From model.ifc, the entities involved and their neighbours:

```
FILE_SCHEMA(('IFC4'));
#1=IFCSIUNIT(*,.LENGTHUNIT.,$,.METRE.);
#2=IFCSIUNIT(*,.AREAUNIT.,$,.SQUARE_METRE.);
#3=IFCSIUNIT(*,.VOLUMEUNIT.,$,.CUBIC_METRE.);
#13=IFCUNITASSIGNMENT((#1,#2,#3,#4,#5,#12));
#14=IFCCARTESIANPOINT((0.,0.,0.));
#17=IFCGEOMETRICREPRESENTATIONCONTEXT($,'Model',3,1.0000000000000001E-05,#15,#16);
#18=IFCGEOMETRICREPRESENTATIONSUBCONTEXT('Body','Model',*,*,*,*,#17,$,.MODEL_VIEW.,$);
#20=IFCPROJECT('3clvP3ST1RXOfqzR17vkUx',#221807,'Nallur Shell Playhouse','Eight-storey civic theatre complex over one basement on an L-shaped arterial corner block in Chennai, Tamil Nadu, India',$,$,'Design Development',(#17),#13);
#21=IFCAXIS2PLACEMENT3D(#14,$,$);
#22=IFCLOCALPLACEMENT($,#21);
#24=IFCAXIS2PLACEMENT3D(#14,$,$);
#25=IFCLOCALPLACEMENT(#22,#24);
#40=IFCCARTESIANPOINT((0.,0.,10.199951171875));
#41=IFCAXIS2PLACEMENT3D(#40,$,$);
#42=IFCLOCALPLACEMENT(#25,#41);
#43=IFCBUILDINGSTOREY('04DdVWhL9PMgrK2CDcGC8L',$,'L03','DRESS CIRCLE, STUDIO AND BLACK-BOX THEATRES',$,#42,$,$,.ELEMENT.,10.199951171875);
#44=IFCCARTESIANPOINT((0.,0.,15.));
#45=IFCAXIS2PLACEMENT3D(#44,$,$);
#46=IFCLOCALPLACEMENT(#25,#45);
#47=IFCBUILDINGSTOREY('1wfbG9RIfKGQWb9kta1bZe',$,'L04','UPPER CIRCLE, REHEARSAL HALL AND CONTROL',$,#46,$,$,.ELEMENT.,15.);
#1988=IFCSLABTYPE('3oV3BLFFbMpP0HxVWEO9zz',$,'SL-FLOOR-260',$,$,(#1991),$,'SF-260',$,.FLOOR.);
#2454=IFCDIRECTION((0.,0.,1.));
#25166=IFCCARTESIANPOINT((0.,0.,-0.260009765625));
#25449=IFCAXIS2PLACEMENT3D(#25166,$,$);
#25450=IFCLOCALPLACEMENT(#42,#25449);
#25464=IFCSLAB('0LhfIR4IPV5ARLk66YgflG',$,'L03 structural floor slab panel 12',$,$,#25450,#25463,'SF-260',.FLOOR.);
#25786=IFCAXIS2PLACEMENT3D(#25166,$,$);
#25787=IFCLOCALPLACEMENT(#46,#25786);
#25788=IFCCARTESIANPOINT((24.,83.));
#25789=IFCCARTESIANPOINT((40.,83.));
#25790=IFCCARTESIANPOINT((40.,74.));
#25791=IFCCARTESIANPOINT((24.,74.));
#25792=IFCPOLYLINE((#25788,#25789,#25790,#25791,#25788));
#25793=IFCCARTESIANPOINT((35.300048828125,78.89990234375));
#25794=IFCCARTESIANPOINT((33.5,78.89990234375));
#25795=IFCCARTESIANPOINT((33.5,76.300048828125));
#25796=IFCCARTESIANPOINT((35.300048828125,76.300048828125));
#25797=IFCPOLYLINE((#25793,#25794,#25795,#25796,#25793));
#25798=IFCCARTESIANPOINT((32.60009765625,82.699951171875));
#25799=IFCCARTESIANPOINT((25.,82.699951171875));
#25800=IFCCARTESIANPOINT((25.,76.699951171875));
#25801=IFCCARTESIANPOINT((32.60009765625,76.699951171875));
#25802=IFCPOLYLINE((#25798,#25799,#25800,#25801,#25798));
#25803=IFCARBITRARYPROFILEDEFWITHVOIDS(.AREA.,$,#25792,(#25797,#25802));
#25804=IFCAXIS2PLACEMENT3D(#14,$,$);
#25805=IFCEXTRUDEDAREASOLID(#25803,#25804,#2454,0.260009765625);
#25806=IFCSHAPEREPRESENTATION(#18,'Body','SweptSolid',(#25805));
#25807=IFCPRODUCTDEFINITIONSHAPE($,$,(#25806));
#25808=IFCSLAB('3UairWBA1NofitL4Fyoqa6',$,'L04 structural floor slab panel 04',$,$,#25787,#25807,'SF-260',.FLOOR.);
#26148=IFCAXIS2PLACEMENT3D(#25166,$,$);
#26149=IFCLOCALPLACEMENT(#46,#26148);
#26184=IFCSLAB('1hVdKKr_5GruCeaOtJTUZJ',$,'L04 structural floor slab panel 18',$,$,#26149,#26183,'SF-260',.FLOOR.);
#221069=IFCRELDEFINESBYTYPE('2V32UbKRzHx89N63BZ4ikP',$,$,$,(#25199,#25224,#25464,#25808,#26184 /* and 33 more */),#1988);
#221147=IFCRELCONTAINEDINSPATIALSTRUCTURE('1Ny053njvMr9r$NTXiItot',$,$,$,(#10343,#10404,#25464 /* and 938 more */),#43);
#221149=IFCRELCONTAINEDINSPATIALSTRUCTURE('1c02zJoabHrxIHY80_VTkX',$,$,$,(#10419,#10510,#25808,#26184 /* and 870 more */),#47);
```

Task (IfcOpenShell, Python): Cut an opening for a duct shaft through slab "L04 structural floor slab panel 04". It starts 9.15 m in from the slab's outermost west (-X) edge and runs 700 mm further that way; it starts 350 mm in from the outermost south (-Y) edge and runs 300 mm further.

```python
import numpy as np
import ifcopenshell
import ifcopenshell.api.feature
import ifcopenshell.api.geometry
import ifcopenshell.api.root
import ifcopenshell.geom
import ifcopenshell.util.placement
import ifcopenshell.util.representation
import ifcopenshell.util.shape
import ifcopenshell.util.unit

model = ifcopenshell.open("model.ifc")
unit_scale = ifcopenshell.util.unit.calculate_unit_scale(model)
settings = ifcopenshell.geom.settings()


def volume(element):
    """Net volume in cubic metres, openings subtracted."""
    shape = ifcopenshell.geom.create_shape(settings, element)
    return ifcopenshell.util.shape.get_volume(shape.geometry)


slab = model.by_id(25808)
before = volume(slab)

# Extent in the slab's own axes, in metres. The edges named are its -X and -Y sides.
slab_shape = ifcopenshell.geom.create_shape(settings, slab)
vertices = ifcopenshell.util.shape.get_vertices(slab_shape.geometry)
x_min, y_min, bottom = vertices.min(axis=0)
top = vertices[:, 2].max()

opening = ifcopenshell.api.root.create_entity(model, ifc_class="IfcOpeningElement", name="Duct shaft opening", predefined_type="OPENING")
context = ifcopenshell.util.representation.get_context(model, "Model", "Body", "MODEL_VIEW")
width, depth = 0.7, 0.3
outline = [(0.0, 0.0), (width, 0.0), (width, depth), (0.0, depth), (0.0, 0.0)]
# Overshoot both faces by 50 mm so the cut is clean.
shape = ifcopenshell.api.geometry.add_slab_representation(
    model, context=context, depth=top - bottom + 0.1, polyline=outline
)
ifcopenshell.api.geometry.assign_representation(model, product=opening, representation=shape)

matrix = ifcopenshell.util.placement.get_local_placement(slab.ObjectPlacement)
matrix[:, 3] = matrix @ np.append(np.array([x_min + 9.15, y_min + 0.35, bottom - 0.05]) / unit_scale, 1.0)
ifcopenshell.api.geometry.edit_object_placement(model, product=opening, matrix=matrix, is_si=False)
ifcopenshell.api.feature.add_feature(model, feature=opening, element=slab)

after = volume(slab)

print(f"slab volume {before:.3f} -> {after:.3f} m3")

model.write("model_edited.ifc")
```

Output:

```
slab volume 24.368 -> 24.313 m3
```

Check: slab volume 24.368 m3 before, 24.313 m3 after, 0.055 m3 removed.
